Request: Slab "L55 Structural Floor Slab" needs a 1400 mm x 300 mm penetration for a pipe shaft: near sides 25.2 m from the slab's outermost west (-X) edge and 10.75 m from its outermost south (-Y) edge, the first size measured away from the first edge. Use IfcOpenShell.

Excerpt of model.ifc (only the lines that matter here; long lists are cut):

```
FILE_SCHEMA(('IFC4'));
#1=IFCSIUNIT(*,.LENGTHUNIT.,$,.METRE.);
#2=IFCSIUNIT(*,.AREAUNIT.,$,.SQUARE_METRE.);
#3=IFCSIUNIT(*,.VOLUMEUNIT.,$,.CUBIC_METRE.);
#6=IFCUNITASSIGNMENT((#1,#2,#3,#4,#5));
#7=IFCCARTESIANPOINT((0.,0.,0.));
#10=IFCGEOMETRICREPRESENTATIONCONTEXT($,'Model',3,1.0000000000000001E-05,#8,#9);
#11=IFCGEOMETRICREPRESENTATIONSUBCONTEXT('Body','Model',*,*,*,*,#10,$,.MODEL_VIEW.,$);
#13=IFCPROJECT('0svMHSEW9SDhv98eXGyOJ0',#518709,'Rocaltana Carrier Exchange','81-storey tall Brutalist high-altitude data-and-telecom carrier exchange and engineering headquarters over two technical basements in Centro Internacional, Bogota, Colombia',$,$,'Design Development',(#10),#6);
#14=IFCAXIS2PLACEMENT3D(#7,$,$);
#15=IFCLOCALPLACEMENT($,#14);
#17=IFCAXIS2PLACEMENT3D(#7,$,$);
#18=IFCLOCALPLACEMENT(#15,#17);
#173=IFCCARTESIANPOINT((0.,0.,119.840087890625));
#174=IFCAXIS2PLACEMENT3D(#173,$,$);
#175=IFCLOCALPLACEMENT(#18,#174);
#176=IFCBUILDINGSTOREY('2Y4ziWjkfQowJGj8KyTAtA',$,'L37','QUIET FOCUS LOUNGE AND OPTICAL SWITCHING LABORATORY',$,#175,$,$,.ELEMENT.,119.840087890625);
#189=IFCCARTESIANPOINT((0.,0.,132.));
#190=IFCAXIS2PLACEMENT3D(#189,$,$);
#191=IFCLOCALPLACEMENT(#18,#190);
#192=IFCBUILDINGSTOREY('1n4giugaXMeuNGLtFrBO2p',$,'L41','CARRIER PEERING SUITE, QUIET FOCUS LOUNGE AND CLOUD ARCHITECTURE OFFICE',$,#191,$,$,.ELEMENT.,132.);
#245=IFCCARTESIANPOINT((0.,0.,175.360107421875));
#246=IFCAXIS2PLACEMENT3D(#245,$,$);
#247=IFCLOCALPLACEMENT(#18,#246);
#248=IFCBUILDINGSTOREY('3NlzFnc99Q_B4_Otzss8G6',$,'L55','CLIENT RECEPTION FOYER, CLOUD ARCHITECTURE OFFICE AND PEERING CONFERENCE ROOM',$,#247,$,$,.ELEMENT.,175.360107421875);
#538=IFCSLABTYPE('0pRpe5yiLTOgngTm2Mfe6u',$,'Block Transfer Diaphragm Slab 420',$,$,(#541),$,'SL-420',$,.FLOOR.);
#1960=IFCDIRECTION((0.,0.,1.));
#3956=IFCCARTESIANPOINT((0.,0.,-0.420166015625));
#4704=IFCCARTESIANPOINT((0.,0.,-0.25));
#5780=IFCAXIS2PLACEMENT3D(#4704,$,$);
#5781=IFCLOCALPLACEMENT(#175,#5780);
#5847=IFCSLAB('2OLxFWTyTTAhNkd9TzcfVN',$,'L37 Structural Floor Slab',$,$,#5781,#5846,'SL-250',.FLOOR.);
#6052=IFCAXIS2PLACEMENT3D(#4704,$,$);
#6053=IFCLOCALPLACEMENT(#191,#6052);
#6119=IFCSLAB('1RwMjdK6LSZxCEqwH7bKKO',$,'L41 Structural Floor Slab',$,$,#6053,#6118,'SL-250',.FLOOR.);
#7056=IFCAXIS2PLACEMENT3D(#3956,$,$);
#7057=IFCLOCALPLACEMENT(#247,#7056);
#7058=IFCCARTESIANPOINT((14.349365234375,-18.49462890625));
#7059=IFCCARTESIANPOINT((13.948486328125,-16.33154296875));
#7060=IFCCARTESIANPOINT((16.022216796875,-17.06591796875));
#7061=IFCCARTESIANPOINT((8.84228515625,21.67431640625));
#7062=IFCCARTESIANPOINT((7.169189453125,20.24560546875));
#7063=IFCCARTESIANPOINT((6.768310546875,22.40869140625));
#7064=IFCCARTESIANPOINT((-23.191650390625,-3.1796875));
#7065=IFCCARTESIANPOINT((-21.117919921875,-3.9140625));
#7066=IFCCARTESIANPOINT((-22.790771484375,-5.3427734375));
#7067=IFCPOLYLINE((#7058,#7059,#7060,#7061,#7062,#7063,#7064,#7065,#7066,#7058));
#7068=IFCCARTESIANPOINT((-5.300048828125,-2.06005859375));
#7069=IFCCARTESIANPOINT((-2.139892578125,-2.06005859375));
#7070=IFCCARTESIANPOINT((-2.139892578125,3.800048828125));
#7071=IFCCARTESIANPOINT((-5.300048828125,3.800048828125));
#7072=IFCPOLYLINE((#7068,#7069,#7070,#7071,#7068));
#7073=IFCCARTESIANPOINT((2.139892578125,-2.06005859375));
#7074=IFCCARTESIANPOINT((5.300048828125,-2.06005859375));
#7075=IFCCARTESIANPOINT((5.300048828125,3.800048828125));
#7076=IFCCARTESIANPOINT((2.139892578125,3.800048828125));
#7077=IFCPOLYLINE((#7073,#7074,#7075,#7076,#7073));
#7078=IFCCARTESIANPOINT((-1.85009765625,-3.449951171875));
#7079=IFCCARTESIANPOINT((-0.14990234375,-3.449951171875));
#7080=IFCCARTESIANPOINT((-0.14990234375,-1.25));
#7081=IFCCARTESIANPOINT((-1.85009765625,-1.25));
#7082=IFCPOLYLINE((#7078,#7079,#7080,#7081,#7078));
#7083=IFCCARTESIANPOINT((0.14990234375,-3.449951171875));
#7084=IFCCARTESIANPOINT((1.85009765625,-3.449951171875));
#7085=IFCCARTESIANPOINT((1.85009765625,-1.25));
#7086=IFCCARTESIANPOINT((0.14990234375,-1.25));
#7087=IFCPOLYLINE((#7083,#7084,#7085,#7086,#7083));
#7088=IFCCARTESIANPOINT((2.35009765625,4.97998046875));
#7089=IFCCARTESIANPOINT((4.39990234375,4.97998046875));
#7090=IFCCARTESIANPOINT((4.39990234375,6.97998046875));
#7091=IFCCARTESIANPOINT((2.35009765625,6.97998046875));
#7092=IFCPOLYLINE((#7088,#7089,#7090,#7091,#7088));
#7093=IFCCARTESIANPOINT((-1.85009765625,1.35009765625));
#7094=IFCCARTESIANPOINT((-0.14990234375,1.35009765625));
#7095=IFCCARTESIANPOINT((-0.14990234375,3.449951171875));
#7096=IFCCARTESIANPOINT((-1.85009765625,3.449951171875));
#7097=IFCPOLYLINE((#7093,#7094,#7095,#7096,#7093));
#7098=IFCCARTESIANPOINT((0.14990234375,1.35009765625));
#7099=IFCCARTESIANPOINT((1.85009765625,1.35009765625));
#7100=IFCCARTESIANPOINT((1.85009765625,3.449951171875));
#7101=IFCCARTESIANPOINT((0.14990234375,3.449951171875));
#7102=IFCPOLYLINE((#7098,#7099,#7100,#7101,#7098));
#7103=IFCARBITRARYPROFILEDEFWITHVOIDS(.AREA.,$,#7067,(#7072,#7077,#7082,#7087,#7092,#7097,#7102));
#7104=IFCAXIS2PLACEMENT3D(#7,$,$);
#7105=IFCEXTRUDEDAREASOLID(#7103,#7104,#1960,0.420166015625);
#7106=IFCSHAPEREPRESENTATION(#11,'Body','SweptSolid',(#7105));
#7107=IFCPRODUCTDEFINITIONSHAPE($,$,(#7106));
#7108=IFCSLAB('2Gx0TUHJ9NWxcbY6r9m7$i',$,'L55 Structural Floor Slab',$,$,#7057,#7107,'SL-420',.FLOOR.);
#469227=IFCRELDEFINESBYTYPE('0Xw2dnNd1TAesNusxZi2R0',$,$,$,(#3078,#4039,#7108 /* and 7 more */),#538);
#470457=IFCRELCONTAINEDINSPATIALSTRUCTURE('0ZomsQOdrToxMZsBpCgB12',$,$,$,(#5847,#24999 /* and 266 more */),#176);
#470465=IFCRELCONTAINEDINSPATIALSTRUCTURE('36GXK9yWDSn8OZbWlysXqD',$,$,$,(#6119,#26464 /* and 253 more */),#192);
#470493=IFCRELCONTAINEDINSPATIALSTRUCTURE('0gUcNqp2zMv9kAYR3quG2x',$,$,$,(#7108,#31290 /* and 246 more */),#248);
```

```python
import numpy as np
import ifcopenshell
import ifcopenshell.api.feature
import ifcopenshell.api.geometry
import ifcopenshell.api.root
import ifcopenshell.geom
import ifcopenshell.util.placement
import ifcopenshell.util.representation
import ifcopenshell.util.shape
import ifcopenshell.util.unit

model = ifcopenshell.open("model.ifc")
unit_scale = ifcopenshell.util.unit.calculate_unit_scale(model)
settings = ifcopenshell.geom.settings()


def volume(element):
    """Net volume in cubic metres, openings subtracted."""
    shape = ifcopenshell.geom.create_shape(settings, element)
    return ifcopenshell.util.shape.get_volume(shape.geometry)


slab = model.by_guid("2Gx0TUHJ9NWxcbY6r9m7$i")
before = volume(slab)

# Extent in the slab's own axes, in metres. The edges named are its -X and -Y sides.
slab_shape = ifcopenshell.geom.create_shape(settings, slab)
vertices = ifcopenshell.util.shape.get_vertices(slab_shape.geometry)
x_min, y_min, bottom = vertices.min(axis=0)
top = vertices[:, 2].max()

opening = ifcopenshell.api.root.create_entity(model, ifc_class="IfcOpeningElement", name="Pipe shaft opening", predefined_type="OPENING")
context = ifcopenshell.util.representation.get_context(model, "Model", "Body", "MODEL_VIEW")
width, depth = 1.4, 0.3
outline = [(0.0, 0.0), (width, 0.0), (width, depth), (0.0, depth), (0.0, 0.0)]
# Overshoot both faces by 50 mm so the cut is clean.
shape = ifcopenshell.api.geometry.add_slab_representation(
    model, context=context, depth=top - bottom + 0.1, polyline=outline
)
ifcopenshell.api.geometry.assign_representation(model, product=opening, representation=shape)

matrix = ifcopenshell.util.placement.get_local_placement(slab.ObjectPlacement)
matrix[:, 3] = matrix @ np.append(np.array([x_min + 25.2, y_min + 10.75, bottom - 0.05]) / unit_scale, 1.0)
ifcopenshell.api.geometry.edit_object_placement(model, product=opening, matrix=matrix, is_si=False)
ifcopenshell.api.feature.add_feature(model, feature=opening, element=slab)

after = volume(slab)

print(f"slab volume {before:.3f} -> {after:.3f} m3")

model.write("model_updated.ifc")
```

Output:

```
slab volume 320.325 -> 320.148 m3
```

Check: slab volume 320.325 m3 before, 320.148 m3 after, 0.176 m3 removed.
